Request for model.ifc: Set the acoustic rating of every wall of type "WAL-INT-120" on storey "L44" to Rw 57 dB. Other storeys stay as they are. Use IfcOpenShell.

First a look at what the model holds.

```python
import ifcopenshell
import ifcopenshell.util.element

model = ifcopenshell.open("model.ifc")
print(model.schema)
storey = next(s for s in model.by_type("IfcBuildingStorey") if s.Name == "L44")
walls = [e for e in ifcopenshell.util.element.get_decomposition(storey) if e.is_a("IfcWall")]
seen = {}
for e in walls:
    element_type = ifcopenshell.util.element.get_type(e)
    key = (element_type.Name if element_type != e and element_type else None, ifcopenshell.util.element.get_pset(e, "Pset_WallCommon", "AcousticRating"))
    seen[key] = seen.get(key, 0) + 1
for (name, value), count in sorted(seen.items(), key=str):
    print(count, "x", name, "|", value)
```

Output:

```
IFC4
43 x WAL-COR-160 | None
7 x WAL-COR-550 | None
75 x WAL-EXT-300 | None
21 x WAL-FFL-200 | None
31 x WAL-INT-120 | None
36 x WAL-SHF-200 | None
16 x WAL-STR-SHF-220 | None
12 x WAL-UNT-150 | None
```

```python
import ifcopenshell
import ifcopenshell.api.pset
import ifcopenshell.util.element

model = ifcopenshell.open("model.ifc")

storey = next(s for s in model.by_type("IfcBuildingStorey") if s.Name == "L44")
walls = [e for e in ifcopenshell.util.element.get_decomposition(storey) if e.is_a("IfcWall")]

count = 0
for e in walls:
    element_type = ifcopenshell.util.element.get_type(e)
    if element_type in (None, e) or element_type.Name != "WAL-INT-120":
        continue
    found = ifcopenshell.util.element.get_pset(e, "Pset_WallCommon", should_inherit=False)
    if found:
        pset = model.by_id(found["id"])
        if len(ifcopenshell.util.element.get_elements_by_pset(pset)) > 1:
            pset = ifcopenshell.api.pset.unshare_pset(model, products=[e], pset=pset)[0]
    else:
        pset = ifcopenshell.api.pset.add_pset(model, product=e, name="Pset_WallCommon")
    ifcopenshell.api.pset.edit_pset(model, pset=pset, properties={"AcousticRating": "Rw 57 dB"})
    count += 1

print(count, "walls updated")

model.write("model-out.ifc")
```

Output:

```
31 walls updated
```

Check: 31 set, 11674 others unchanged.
